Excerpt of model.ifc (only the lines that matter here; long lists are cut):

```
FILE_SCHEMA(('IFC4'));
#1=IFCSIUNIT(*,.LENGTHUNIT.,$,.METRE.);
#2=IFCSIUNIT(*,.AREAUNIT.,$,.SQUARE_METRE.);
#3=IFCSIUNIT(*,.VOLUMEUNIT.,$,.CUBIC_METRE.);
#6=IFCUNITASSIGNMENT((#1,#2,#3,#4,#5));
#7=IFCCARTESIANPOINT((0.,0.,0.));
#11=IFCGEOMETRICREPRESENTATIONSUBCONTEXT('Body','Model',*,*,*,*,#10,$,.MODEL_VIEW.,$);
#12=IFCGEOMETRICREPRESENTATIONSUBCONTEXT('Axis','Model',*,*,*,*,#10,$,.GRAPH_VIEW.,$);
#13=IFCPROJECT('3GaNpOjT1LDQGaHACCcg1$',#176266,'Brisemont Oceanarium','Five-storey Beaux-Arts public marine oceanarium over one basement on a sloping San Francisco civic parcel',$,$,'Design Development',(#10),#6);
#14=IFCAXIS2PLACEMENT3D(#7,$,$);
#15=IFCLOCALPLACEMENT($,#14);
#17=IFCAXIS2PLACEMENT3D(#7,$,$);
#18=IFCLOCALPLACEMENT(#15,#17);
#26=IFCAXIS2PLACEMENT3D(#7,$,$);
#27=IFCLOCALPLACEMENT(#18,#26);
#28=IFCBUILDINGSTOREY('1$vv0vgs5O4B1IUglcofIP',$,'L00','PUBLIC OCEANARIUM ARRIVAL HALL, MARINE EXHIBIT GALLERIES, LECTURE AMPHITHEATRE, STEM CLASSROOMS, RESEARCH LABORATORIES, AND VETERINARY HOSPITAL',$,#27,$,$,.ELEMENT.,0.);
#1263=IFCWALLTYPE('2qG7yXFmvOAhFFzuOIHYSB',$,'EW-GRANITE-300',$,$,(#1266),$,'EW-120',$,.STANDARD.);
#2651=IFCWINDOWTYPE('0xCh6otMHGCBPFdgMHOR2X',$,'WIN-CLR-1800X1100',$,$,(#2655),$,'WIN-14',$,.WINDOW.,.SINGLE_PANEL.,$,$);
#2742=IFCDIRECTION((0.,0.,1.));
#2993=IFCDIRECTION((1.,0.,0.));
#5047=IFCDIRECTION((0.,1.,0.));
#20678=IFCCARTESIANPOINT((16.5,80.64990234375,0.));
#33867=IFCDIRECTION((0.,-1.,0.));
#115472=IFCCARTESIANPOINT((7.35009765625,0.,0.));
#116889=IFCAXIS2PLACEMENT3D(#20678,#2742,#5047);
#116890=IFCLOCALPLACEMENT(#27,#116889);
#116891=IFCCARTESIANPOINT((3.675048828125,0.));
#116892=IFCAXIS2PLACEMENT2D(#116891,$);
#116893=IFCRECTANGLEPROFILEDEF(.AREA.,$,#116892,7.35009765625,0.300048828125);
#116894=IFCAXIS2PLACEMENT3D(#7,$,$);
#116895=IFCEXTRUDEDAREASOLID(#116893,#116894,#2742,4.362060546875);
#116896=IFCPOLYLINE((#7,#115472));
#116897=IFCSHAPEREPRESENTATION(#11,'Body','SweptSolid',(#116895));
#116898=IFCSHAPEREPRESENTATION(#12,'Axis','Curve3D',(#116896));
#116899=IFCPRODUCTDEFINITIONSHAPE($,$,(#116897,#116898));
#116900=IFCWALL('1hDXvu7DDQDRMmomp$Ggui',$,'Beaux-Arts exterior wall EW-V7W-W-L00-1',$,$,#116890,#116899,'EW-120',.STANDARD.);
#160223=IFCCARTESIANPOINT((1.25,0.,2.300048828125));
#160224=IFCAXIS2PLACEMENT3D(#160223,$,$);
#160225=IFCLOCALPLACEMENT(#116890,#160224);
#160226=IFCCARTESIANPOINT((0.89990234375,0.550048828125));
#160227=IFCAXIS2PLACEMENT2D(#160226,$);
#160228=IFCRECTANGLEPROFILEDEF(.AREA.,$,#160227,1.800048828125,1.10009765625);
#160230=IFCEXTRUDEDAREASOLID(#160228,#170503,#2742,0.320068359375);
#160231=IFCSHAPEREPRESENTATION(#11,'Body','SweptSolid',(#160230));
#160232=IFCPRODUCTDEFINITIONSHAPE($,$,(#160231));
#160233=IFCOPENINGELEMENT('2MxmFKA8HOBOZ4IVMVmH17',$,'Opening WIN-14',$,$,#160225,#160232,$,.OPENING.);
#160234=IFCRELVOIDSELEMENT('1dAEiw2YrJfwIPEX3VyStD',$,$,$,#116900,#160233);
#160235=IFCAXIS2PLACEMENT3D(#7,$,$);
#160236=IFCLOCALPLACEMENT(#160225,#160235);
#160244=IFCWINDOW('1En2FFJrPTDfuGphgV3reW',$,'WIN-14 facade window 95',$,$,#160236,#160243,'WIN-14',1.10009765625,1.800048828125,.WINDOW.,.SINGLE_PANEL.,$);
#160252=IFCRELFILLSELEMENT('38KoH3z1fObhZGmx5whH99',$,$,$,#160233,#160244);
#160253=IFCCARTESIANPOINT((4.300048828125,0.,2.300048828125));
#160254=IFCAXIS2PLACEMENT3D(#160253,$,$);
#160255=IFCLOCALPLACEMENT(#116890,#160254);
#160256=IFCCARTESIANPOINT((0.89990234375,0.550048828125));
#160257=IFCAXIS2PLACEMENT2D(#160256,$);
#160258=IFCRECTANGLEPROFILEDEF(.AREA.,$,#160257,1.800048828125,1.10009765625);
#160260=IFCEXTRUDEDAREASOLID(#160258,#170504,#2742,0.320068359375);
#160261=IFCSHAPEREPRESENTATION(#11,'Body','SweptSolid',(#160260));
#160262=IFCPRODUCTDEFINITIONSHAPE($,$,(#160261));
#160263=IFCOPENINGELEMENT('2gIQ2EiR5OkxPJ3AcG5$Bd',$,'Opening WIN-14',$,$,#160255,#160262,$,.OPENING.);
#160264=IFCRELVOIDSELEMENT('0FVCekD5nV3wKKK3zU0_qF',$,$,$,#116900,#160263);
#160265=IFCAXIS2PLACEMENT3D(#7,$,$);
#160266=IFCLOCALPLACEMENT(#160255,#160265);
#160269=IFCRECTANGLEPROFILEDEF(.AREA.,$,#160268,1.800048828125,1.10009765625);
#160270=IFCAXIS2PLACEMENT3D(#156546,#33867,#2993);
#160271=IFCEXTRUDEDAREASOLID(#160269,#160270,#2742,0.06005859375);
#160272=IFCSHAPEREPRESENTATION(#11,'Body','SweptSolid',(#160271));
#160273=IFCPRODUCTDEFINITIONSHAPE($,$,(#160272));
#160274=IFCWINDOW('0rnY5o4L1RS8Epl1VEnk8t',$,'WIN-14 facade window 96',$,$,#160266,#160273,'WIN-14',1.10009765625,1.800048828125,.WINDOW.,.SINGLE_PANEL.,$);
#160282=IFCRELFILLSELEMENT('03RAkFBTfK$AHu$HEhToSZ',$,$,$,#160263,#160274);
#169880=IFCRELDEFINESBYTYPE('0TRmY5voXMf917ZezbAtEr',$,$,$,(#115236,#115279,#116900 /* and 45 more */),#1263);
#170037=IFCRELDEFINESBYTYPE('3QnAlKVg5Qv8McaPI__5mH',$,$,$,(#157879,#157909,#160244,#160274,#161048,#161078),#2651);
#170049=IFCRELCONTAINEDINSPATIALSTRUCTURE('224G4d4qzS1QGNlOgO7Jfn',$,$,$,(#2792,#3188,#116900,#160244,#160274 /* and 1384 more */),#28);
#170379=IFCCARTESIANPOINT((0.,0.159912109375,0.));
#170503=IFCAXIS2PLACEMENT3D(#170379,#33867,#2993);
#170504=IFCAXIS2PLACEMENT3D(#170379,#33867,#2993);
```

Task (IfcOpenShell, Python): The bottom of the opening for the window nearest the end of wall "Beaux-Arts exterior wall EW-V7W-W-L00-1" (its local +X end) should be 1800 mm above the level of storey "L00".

```python
import numpy as np
import ifcopenshell
import ifcopenshell.api.geometry
import ifcopenshell.geom
import ifcopenshell.util.element
import ifcopenshell.util.placement
import ifcopenshell.util.shape
import ifcopenshell.util.unit

model = ifcopenshell.open("model.ifc")
unit_scale = ifcopenshell.util.unit.calculate_unit_scale(model)

window = model.by_guid("0rnY5o4L1RS8Epl1VEnk8t")
opening = window.FillsVoids[0].RelatingOpeningElement
storey = ifcopenshell.util.element.get_container(window, ifc_class="IfcBuildingStorey")
level = ifcopenshell.util.placement.get_local_placement(storey.ObjectPlacement)[2, 3]

# The opening's origin need not be at the sill, so measure its lowest point.
shape = ifcopenshell.geom.create_shape(ifcopenshell.geom.settings(), opening)
bottom = ifcopenshell.util.shape.get_shape_bottom_elevation(shape, shape.geometry) / unit_scale
dz = level + 1.8 - bottom

shift = np.array([0.0, 0.0, dz])
# The window is placed relative to its opening, so it follows when the opening moves.
matrix = ifcopenshell.util.placement.get_local_placement(opening.ObjectPlacement)
matrix[:3, 3] += shift
ifcopenshell.api.geometry.edit_object_placement(
    model, product=opening, matrix=matrix, is_si=False, should_transform_children=True
)

print(f"moved by {dz * unit_scale:+.3f} m")

model.write("model-out.ifc")
```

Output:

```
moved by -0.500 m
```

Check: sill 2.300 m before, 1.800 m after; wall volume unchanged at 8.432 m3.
